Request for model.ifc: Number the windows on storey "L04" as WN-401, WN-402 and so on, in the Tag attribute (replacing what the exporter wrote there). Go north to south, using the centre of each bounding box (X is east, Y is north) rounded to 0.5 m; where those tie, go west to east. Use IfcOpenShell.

First a look at what the model holds.

```python
import ifcopenshell
import ifcopenshell.util.element
import ifcopenshell.util.placement

model = ifcopenshell.open("model.ifc")
print(model.schema)
storey = next(s for s in model.by_type("IfcBuildingStorey") if s.Name == "L04")
windows = [e for e in ifcopenshell.util.element.get_decomposition(storey) if e.is_a("IfcWindow")]
for e in sorted(windows, key=lambda e: e.id()):
    origin = ifcopenshell.util.placement.get_local_placement(e.ObjectPlacement)[:3, 3]
    print(e.id(), e.Tag, e.Name, origin.round(2) + 0.0, sep=" | ")
```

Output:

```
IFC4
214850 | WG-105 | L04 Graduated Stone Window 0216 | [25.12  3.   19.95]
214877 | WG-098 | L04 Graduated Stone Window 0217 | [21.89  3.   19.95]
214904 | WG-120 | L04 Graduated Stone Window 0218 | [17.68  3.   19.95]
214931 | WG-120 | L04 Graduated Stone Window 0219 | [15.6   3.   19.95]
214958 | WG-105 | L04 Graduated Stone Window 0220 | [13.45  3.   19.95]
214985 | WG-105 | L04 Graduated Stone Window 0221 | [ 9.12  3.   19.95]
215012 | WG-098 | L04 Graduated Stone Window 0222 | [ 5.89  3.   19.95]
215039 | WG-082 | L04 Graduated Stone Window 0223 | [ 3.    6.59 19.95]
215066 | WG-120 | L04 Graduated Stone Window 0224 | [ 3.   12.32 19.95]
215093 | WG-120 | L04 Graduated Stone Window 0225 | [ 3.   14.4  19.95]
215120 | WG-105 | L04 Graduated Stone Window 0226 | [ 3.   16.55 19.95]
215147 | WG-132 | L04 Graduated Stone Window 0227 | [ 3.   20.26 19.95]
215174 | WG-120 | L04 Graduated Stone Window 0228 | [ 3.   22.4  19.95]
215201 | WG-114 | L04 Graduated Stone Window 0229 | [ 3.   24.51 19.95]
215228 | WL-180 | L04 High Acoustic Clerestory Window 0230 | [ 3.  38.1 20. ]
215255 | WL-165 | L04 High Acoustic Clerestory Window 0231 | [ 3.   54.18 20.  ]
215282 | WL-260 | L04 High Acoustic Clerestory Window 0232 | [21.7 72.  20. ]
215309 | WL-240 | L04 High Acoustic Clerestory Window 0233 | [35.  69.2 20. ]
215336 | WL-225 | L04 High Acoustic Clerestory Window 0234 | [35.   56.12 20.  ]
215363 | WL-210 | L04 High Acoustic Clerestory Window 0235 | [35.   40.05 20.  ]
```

```python
import ifcopenshell
import ifcopenshell.geom
import ifcopenshell.util.element
import ifcopenshell.util.shape

model = ifcopenshell.open("model.ifc")
settings = ifcopenshell.geom.settings()
settings.set("use-world-coords", True)


def centre(element):
    shape = ifcopenshell.geom.create_shape(settings, element)
    return ifcopenshell.util.shape.get_bbox_centroid(shape.geometry)


storey = next(s for s in model.by_type("IfcBuildingStorey") if s.Name == "L04")
windows = [e for e in ifcopenshell.util.element.get_decomposition(storey) if e.is_a("IfcWindow")]

# Insertion points can sit at a corner or the storey origin, so sort by the geometry (in metres).
centres = {e: centre(e) for e in windows}
windows.sort(key=lambda e: (-round(centres[e][1] / 0.5), centres[e][0]))

for i, e in enumerate(windows, start=1):
    number = f"WN-4{i:02d}"
    e.Tag = number
    print(e.id(), number)

model.write("model_v2.ifc")
```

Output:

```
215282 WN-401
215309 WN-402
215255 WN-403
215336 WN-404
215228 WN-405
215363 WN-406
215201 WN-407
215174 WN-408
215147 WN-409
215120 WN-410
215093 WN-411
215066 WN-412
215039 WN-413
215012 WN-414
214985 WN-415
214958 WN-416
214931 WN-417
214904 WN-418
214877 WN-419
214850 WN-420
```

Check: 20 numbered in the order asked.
